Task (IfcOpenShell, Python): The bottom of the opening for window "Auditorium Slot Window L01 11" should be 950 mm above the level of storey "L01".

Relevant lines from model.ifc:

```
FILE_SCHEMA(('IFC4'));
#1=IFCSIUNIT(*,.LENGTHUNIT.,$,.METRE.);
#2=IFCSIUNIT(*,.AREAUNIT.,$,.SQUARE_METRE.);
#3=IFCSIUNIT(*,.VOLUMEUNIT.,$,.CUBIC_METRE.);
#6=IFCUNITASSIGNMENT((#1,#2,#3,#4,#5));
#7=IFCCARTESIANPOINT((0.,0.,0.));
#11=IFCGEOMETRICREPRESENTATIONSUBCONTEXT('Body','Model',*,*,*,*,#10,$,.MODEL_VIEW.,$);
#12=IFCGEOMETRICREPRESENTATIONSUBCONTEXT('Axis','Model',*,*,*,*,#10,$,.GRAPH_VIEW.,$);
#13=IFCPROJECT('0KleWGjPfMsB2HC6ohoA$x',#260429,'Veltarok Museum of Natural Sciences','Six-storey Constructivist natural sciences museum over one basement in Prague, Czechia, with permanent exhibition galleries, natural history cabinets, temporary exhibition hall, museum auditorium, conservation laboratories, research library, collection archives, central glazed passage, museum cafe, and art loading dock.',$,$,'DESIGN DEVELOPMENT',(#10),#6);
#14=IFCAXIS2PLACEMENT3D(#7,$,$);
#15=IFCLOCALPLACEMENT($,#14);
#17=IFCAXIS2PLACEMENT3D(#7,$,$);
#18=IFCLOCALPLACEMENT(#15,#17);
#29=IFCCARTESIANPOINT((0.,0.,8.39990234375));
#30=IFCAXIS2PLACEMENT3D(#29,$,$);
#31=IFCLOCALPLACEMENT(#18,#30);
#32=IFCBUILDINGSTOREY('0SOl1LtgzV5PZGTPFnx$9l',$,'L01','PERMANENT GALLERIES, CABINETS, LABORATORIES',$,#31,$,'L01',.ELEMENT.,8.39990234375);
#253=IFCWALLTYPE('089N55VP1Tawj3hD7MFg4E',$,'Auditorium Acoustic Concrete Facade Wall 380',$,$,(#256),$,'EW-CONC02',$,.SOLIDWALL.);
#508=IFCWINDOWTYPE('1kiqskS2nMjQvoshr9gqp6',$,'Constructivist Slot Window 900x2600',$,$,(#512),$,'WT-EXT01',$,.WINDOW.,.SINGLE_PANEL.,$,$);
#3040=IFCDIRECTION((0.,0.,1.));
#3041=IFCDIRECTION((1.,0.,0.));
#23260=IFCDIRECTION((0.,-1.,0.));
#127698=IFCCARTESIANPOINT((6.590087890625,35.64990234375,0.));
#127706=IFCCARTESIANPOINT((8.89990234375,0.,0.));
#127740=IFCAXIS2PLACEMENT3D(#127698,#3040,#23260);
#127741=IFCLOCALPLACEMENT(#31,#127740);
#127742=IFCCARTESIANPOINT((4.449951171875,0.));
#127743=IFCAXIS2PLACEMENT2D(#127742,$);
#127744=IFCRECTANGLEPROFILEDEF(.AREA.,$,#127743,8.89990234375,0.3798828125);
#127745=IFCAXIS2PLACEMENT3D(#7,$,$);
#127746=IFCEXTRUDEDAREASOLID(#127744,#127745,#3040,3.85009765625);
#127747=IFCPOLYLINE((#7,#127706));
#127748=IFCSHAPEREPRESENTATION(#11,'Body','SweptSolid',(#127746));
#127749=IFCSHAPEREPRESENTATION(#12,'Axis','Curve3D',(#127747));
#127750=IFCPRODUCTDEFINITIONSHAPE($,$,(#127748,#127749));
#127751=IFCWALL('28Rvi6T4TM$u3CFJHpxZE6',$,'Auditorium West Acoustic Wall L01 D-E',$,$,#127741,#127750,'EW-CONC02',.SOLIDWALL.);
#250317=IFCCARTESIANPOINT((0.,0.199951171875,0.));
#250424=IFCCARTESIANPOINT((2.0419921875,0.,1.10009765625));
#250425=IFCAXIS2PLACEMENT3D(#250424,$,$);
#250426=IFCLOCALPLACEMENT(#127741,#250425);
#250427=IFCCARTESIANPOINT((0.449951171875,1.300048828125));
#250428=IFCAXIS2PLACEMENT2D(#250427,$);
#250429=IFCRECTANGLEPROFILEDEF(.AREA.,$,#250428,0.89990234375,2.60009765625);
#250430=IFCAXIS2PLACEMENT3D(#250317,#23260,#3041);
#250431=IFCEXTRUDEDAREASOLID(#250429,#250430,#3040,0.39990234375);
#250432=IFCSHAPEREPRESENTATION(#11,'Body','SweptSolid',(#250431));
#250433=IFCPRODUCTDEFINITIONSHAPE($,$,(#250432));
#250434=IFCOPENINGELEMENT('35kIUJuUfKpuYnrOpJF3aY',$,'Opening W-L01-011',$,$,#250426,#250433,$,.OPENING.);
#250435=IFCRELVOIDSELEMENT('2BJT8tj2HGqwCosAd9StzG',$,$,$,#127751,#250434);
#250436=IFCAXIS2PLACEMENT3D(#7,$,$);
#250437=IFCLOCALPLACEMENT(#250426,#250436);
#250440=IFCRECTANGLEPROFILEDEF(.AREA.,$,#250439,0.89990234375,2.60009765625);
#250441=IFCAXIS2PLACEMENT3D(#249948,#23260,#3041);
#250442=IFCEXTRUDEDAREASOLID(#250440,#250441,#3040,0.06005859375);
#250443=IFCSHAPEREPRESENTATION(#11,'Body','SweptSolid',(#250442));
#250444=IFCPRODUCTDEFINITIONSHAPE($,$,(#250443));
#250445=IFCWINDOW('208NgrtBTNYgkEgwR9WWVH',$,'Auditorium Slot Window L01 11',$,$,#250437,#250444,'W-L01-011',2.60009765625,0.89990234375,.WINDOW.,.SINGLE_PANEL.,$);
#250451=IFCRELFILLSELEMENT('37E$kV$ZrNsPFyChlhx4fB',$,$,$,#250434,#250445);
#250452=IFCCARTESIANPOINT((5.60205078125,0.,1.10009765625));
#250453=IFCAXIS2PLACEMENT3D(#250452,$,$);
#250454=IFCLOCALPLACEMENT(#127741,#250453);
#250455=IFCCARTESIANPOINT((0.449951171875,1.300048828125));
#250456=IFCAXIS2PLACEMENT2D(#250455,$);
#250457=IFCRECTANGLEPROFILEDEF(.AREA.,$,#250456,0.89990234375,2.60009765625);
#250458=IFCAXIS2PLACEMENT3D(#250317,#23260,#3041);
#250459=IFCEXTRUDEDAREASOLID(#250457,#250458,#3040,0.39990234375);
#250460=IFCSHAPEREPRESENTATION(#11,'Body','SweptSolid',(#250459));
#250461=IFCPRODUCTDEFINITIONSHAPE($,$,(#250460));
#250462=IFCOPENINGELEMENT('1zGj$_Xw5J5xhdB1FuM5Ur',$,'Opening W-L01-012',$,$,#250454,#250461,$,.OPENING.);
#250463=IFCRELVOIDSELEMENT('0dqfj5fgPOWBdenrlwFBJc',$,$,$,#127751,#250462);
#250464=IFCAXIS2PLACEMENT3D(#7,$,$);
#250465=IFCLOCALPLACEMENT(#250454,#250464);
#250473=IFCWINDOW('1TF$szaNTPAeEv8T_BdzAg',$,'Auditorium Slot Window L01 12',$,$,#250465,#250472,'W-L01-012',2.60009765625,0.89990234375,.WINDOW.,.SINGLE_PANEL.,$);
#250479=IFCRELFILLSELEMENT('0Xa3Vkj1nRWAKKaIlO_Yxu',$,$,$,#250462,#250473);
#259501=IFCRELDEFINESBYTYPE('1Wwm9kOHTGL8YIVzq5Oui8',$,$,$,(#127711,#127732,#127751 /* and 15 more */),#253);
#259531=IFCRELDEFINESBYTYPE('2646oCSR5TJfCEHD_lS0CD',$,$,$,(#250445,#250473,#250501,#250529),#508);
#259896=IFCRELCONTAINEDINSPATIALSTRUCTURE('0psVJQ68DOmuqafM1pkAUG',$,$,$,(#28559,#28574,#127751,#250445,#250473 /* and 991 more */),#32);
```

```python
import numpy as np
import ifcopenshell
import ifcopenshell.api.geometry
import ifcopenshell.geom
import ifcopenshell.util.element
import ifcopenshell.util.placement
import ifcopenshell.util.shape
import ifcopenshell.util.unit

model = ifcopenshell.open("model.ifc")
unit_scale = ifcopenshell.util.unit.calculate_unit_scale(model)

window = model.by_guid("208NgrtBTNYgkEgwR9WWVH")
opening = window.FillsVoids[0].RelatingOpeningElement
storey = ifcopenshell.util.element.get_container(window, ifc_class="IfcBuildingStorey")
level = ifcopenshell.util.placement.get_local_placement(storey.ObjectPlacement)[2, 3]

# The opening's origin need not be at the sill, so measure its lowest point.
shape = ifcopenshell.geom.create_shape(ifcopenshell.geom.settings(), opening)
bottom = ifcopenshell.util.shape.get_shape_bottom_elevation(shape, shape.geometry) / unit_scale
dz = level + 0.95 / unit_scale - bottom

shift = np.array([0.0, 0.0, dz])
# The window is placed relative to its opening, so it follows when the opening moves.
matrix = ifcopenshell.util.placement.get_local_placement(opening.ObjectPlacement)
matrix[:3, 3] += shift
ifcopenshell.api.geometry.edit_object_placement(
    model, product=opening, matrix=matrix, is_si=False, should_transform_children=True
)

print(f"moved by {dz * unit_scale:+.3f} m")

model.write("model-out.ifc")
```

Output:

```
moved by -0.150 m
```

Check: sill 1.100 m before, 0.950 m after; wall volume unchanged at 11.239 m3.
